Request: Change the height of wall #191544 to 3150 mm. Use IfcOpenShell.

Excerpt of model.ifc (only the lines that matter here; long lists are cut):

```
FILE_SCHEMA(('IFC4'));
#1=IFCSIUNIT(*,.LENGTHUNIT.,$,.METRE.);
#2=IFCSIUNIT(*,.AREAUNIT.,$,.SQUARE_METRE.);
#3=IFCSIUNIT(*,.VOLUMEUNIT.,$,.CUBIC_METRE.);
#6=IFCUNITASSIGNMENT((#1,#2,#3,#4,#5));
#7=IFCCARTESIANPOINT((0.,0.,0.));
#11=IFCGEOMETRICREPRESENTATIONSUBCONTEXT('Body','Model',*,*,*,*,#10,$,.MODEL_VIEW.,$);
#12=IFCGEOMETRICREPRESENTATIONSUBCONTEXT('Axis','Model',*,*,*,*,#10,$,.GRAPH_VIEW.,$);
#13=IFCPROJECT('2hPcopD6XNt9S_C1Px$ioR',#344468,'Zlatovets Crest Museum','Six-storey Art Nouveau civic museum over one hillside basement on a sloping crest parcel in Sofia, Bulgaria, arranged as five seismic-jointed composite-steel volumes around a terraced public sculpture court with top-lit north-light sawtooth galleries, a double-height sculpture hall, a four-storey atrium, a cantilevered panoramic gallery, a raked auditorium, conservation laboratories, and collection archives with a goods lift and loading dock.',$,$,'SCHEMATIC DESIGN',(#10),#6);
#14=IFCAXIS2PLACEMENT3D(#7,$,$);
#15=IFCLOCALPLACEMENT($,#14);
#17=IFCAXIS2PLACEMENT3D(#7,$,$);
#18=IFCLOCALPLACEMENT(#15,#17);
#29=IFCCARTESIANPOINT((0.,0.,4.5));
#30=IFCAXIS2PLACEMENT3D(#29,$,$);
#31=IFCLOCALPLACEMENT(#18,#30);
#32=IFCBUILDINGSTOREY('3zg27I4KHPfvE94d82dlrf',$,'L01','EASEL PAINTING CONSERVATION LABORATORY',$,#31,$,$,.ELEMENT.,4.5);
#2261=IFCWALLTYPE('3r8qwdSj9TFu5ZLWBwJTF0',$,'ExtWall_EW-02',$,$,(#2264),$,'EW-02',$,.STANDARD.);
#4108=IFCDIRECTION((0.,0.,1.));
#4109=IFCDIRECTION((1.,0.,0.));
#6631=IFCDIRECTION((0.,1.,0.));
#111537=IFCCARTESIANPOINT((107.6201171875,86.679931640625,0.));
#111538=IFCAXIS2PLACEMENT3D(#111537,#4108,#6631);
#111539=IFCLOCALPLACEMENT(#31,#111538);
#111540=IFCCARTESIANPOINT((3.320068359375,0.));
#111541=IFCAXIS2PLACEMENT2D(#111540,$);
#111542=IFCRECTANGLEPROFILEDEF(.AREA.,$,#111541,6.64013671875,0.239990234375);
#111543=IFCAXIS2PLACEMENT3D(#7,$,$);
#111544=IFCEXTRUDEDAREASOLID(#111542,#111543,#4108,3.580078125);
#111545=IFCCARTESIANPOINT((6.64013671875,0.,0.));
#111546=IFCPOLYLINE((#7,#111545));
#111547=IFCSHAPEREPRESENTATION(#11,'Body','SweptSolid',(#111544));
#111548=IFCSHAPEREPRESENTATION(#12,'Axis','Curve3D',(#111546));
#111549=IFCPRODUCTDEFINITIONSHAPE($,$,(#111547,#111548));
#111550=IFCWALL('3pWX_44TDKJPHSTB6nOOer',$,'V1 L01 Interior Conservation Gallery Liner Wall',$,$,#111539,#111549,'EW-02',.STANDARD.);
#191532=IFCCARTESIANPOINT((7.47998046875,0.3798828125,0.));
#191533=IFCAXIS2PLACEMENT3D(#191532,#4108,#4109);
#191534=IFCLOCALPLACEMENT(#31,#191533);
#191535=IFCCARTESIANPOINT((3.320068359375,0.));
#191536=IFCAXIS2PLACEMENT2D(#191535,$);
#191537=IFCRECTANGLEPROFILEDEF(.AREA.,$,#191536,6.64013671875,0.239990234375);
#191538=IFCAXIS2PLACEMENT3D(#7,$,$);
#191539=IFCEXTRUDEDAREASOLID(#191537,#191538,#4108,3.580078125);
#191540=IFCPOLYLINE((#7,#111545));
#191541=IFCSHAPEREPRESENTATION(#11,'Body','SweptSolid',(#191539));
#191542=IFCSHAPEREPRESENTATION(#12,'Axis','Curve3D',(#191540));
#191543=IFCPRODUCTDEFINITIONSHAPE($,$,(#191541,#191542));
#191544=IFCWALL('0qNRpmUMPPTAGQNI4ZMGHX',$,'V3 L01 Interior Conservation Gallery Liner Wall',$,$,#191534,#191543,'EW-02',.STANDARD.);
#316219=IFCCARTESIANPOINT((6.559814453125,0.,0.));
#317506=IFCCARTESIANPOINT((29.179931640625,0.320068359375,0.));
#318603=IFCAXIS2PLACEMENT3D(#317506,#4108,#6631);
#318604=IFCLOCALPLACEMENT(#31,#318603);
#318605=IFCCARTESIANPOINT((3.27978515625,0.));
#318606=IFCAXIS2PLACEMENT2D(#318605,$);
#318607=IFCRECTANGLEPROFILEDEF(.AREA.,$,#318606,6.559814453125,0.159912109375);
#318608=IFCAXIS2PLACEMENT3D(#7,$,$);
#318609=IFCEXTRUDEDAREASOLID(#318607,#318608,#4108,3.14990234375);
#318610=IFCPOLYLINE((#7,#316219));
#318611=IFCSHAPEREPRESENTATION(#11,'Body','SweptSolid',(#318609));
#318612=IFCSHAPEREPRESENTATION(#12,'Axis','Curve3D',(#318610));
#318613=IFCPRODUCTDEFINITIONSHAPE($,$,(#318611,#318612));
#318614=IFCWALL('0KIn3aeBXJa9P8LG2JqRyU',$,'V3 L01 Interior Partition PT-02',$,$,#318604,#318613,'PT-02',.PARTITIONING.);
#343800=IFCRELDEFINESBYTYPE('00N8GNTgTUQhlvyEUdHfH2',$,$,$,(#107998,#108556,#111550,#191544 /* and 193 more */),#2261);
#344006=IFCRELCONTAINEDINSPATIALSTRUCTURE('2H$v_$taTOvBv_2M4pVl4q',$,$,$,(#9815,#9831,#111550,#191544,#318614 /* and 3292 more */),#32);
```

```python
import ifcopenshell
import ifcopenshell.geom
import ifcopenshell.util.representation
import ifcopenshell.util.shape
import ifcopenshell.util.unit

model = ifcopenshell.open("model.ifc")
unit_scale = ifcopenshell.util.unit.calculate_unit_scale(model)
settings = ifcopenshell.geom.settings()


def volume(element):
    """Net volume in cubic metres, openings subtracted."""
    shape = ifcopenshell.geom.create_shape(settings, element)
    return ifcopenshell.util.shape.get_volume(shape.geometry)


wall = model.by_guid("0qNRpmUMPPTAGQNI4ZMGHX")
before = volume(wall)

body = ifcopenshell.util.representation.get_representation(wall, "Model", "Body")
solid = body.Items[0]
old_height = solid.Depth
solid.Depth = 3.15 / unit_scale
after = volume(wall)

print(f"height {old_height:g} -> {solid.Depth:g}, volume {before:.3f} -> {after:.3f} m3")

model.write("model_v2.ifc")
```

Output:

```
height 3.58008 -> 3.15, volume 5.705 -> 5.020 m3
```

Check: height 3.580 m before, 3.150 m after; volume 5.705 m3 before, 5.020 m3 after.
